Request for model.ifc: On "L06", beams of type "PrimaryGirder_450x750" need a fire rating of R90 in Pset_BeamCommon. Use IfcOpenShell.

First a look at what the model holds.

```python
import ifcopenshell
import ifcopenshell.util.element

model = ifcopenshell.open("model.ifc")
print(model.schema)
storey = next(s for s in model.by_type("IfcBuildingStorey") if s.Name == "L06")
beams = [e for e in ifcopenshell.util.element.get_decomposition(storey) if e.is_a("IfcBeam")]
seen = {}
for e in beams:
    element_type = ifcopenshell.util.element.get_type(e)
    key = (element_type.Name if element_type != e and element_type else None, ifcopenshell.util.element.get_pset(e, "Pset_BeamCommon", "FireRating"))
    seen[key] = seen.get(key, 0) + 1
for (name, value), count in sorted(seen.items(), key=str):
    print(count, "x", name, "|", value)
```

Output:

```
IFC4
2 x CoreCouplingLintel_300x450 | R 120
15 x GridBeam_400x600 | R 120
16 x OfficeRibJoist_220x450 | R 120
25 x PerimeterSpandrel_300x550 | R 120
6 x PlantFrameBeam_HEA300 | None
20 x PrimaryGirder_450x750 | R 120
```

```python
import ifcopenshell
import ifcopenshell.api.pset
import ifcopenshell.util.element

model = ifcopenshell.open("model.ifc")

storey = next(s for s in model.by_type("IfcBuildingStorey") if s.Name == "L06")
beams = [e for e in ifcopenshell.util.element.get_decomposition(storey) if e.is_a("IfcBeam")]

count = 0
for e in beams:
    element_type = ifcopenshell.util.element.get_type(e)
    if element_type in (None, e) or element_type.Name != "PrimaryGirder_450x750":
        continue
    # add_pset returns the element's existing set when there is one.
    pset = ifcopenshell.api.pset.add_pset(model, product=e, name="Pset_BeamCommon")
    ifcopenshell.api.pset.edit_pset(model, pset=pset, properties={"FireRating": "R90"})
    count += 1

print(count, "beams updated")

model.write("model_edited.ifc")
```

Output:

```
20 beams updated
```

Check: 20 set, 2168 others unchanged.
